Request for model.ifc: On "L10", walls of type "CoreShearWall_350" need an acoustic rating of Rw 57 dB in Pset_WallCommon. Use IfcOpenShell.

First a look at what the model holds.

```python
import ifcopenshell
import ifcopenshell.util.element

model = ifcopenshell.open("model.ifc")
print(model.schema)
storey = next(s for s in model.by_type("IfcBuildingStorey") if s.Name == "L10")
walls = [e for e in ifcopenshell.util.element.get_decomposition(storey) if e.is_a("IfcWall")]
seen = {}
for e in walls:
    element_type = ifcopenshell.util.element.get_type(e)
    key = (element_type.Name if element_type != e and element_type else None, ifcopenshell.util.element.get_pset(e, "Pset_WallCommon", "AcousticRating"))
    seen[key] = seen.get(key, 0) + 1
for (name, value), count in sorted(seen.items(), key=str):
    print(count, "x", name, "|", value)
```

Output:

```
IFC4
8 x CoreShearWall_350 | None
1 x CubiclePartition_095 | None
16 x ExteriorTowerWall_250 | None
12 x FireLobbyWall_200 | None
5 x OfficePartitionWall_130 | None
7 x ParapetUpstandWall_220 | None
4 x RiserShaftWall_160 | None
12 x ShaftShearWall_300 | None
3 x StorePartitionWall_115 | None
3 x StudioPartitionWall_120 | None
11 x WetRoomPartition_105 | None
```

```python
import ifcopenshell
import ifcopenshell.api.pset
import ifcopenshell.util.element

model = ifcopenshell.open("model.ifc")

storey = next(s for s in model.by_type("IfcBuildingStorey") if s.Name == "L10")
walls = [e for e in ifcopenshell.util.element.get_decomposition(storey) if e.is_a("IfcWall")]

count = 0
for e in walls:
    element_type = ifcopenshell.util.element.get_type(e)
    if element_type in (None, e) or element_type.Name != "CoreShearWall_350":
        continue
    # add_pset returns the element's existing set when there is one.
    pset = ifcopenshell.api.pset.add_pset(model, product=e, name="Pset_WallCommon")
    ifcopenshell.api.pset.edit_pset(model, pset=pset, properties={"AcousticRating": "Rw 57 dB"})
    count += 1

print(count, "walls updated")

model.write("model_rev.ifc")
```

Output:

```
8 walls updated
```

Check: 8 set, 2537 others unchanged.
